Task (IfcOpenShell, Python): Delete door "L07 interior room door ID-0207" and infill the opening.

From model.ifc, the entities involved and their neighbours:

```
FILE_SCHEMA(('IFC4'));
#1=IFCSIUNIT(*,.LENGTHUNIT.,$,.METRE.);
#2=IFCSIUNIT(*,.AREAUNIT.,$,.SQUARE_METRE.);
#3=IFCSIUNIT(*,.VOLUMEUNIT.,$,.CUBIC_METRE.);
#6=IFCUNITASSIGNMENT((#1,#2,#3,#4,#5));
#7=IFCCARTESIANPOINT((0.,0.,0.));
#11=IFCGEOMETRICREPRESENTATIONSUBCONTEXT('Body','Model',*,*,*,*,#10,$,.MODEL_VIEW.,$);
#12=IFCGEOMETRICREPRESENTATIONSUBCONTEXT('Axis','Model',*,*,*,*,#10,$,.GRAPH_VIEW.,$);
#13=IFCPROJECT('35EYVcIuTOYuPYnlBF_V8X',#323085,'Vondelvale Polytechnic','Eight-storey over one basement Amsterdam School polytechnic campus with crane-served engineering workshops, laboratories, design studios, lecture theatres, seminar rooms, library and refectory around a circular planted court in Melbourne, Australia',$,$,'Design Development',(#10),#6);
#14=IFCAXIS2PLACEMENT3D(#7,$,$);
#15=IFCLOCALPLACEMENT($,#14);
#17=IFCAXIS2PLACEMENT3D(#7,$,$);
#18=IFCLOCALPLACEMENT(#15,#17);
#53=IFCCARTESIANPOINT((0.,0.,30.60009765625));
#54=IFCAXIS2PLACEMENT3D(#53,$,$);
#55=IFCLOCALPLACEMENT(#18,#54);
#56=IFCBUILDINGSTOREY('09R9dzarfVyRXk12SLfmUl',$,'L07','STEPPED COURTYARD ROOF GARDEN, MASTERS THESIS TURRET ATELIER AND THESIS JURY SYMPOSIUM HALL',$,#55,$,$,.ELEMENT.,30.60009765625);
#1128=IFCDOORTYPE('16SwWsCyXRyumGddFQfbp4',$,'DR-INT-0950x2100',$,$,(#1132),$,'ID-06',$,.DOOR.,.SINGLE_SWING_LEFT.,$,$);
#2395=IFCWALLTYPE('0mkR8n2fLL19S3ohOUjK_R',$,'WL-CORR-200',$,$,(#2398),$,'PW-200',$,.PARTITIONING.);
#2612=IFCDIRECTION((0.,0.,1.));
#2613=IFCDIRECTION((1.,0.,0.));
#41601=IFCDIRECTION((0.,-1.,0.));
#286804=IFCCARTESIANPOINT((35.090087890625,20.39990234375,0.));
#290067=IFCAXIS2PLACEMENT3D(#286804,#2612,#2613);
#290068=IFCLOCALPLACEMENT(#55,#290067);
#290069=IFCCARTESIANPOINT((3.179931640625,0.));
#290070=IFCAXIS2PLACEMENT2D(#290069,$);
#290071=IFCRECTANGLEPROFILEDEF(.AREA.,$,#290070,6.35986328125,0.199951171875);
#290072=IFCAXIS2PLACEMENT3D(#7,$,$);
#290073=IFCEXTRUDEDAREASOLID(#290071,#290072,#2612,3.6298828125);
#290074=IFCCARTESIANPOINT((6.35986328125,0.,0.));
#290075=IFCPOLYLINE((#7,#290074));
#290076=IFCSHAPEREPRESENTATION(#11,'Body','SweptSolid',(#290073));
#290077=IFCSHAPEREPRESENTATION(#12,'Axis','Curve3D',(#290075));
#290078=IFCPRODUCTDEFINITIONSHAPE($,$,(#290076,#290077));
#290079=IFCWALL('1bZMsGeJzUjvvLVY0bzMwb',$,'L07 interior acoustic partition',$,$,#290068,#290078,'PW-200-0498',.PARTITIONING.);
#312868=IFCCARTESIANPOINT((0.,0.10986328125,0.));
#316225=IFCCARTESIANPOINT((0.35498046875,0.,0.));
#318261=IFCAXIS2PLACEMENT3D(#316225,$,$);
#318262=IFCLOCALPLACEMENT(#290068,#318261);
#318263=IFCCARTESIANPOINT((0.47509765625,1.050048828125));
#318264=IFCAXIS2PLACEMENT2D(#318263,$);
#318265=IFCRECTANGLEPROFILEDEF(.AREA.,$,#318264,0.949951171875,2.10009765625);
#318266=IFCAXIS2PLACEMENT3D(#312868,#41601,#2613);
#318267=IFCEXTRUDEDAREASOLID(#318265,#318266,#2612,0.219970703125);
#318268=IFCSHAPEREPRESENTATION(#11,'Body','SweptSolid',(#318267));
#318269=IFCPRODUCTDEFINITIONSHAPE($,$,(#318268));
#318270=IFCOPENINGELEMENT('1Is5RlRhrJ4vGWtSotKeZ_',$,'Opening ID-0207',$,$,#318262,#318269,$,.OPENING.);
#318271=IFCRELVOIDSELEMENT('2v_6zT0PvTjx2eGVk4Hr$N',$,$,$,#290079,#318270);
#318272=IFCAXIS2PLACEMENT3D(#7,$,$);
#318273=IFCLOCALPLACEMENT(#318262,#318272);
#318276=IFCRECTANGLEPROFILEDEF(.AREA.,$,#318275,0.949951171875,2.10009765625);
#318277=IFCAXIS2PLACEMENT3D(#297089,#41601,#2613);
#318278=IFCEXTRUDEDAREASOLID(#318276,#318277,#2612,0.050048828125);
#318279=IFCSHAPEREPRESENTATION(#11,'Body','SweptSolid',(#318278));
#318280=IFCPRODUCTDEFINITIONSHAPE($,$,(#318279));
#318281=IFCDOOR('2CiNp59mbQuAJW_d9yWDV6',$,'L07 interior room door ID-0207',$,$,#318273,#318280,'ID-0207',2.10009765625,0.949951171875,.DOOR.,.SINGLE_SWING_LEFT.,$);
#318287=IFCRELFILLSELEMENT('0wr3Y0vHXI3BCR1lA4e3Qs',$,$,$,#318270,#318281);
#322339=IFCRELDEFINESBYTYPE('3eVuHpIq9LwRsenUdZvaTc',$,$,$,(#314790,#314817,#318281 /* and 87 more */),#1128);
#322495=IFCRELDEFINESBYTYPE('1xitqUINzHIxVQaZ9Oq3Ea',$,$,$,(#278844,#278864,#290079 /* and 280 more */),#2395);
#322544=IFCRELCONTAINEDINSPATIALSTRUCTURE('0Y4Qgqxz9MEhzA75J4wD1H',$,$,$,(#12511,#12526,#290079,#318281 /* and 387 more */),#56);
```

```python
import ifcopenshell
import ifcopenshell.api.feature
import ifcopenshell.api.root
import ifcopenshell.geom
import ifcopenshell.util.shape

model = ifcopenshell.open("model.ifc")
settings = ifcopenshell.geom.settings()


def volume(element):
    """Net volume in cubic metres, openings subtracted."""
    shape = ifcopenshell.geom.create_shape(settings, element)
    return ifcopenshell.util.shape.get_volume(shape.geometry)


door = model.by_guid("2CiNp59mbQuAJW_d9yWDV6")
opening = door.FillsVoids[0].RelatingOpeningElement
wall = opening.VoidsElements[0].RelatingBuildingElement
before = volume(wall)

ifcopenshell.api.root.remove_product(model, product=door)
ifcopenshell.api.feature.remove_feature(model, feature=opening)

after = volume(wall)

print(f"wall volume {before:.3f} -> {after:.3f} m3")

model.write("model_edited.ifc")
```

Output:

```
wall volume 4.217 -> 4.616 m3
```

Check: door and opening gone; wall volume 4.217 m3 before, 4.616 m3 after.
